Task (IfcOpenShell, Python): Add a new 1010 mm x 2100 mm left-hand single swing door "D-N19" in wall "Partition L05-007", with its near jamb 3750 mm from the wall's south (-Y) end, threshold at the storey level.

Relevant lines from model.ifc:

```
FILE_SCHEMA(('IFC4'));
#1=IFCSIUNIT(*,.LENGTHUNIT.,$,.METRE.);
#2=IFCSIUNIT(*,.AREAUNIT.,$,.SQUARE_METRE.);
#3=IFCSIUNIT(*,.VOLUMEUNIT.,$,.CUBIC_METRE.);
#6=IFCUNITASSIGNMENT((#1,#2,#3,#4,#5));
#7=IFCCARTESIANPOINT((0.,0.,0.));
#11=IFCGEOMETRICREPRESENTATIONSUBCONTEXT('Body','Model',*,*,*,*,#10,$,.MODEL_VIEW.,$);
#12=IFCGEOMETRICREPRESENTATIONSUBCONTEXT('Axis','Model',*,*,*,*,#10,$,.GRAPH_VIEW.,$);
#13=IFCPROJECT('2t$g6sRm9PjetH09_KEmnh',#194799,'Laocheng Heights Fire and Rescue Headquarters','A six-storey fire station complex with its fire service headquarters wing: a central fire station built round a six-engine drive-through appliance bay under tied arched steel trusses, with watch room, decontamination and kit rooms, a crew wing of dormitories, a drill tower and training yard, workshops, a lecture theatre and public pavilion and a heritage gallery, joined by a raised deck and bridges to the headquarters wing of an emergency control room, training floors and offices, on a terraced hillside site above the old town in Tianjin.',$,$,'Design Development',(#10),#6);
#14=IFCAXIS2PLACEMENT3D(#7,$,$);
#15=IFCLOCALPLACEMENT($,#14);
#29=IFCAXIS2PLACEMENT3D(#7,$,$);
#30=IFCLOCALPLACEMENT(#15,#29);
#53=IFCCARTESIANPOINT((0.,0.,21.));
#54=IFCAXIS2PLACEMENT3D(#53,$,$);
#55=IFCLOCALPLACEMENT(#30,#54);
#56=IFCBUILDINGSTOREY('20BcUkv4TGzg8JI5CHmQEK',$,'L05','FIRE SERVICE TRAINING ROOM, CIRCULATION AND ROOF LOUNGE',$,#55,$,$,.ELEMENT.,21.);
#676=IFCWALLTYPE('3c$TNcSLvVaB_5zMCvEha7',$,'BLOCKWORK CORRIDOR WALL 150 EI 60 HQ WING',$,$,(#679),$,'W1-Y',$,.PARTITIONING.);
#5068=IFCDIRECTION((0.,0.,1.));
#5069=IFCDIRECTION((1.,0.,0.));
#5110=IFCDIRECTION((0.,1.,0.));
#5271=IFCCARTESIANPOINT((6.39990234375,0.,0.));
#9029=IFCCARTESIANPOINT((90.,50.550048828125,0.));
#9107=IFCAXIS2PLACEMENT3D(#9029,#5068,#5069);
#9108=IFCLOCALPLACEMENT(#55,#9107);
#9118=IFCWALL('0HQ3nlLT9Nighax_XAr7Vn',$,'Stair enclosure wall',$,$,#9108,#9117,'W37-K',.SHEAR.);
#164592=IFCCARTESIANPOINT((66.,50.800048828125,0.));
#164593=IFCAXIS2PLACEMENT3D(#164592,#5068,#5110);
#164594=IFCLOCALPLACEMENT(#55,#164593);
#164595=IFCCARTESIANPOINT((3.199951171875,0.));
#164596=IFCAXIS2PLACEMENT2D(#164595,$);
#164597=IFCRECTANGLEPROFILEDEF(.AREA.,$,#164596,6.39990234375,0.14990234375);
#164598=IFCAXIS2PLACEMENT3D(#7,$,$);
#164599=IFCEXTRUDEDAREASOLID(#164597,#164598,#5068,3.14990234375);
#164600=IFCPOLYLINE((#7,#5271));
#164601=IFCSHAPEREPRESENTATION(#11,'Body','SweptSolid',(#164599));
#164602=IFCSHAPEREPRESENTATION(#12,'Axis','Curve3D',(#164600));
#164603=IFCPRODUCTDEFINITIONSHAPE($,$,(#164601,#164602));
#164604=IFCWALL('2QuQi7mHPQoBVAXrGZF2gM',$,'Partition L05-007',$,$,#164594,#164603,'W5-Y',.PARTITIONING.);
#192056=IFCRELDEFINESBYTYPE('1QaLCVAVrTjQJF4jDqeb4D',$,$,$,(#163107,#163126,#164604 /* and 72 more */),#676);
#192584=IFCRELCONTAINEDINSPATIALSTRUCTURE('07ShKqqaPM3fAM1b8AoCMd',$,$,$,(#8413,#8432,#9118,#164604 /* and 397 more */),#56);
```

```python
import numpy as np
import ifcopenshell
import ifcopenshell.api.feature
import ifcopenshell.api.geometry
import ifcopenshell.api.root
import ifcopenshell.api.spatial
import ifcopenshell.geom
import ifcopenshell.util.element
import ifcopenshell.util.placement
import ifcopenshell.util.representation
import ifcopenshell.util.shape
import ifcopenshell.util.unit

model = ifcopenshell.open("model.ifc")
unit_scale = ifcopenshell.util.unit.calculate_unit_scale(model)
settings = ifcopenshell.geom.settings()


def volume(element):
    """Net volume in cubic metres, openings subtracted."""
    shape = ifcopenshell.geom.create_shape(settings, element)
    return ifcopenshell.util.shape.get_volume(shape.geometry)


wall = model.by_guid("2QuQi7mHPQoBVAXrGZF2gM")
storey = ifcopenshell.util.element.get_container(wall, ifc_class="IfcBuildingStorey")
context = ifcopenshell.util.representation.get_context(model, "Model", "Body", "MODEL_VIEW")
before = volume(wall)

width, height, from_end, sill = 1.01, 2.1, 3.75, 0.0  # metres

# The wall runs along its own X axis, and the end named is its -X end.
wall_shape = ifcopenshell.geom.create_shape(settings, wall)
x, y, z = ifcopenshell.util.shape.get_vertices(wall_shape.geometry).T
start = x.min() + from_end
face, thickness = float(y.min()), float(y.max() - y.min())
wall_matrix = ifcopenshell.util.placement.get_local_placement(wall.ObjectPlacement)
level = ifcopenshell.util.placement.get_local_placement(storey.ObjectPlacement)[2, 3]


def in_wall(x, y):
    """Placement at x, y metres in the wall's axes, at sill height."""
    matrix = wall_matrix.copy()
    matrix[:, 3] = wall_matrix @ np.array([x / unit_scale, y / unit_scale, 0.0, 1.0])
    matrix[2, 3] = level + sill / unit_scale
    return matrix


# Opening: a box that overshoots both wall faces by 50 mm.
opening = ifcopenshell.api.root.create_entity(model, ifc_class="IfcOpeningElement", predefined_type="OPENING")
box = ifcopenshell.api.geometry.add_wall_representation(
    model, context=context, length=width, height=height, thickness=thickness + 0.1
)
ifcopenshell.api.geometry.assign_representation(model, product=opening, representation=box)
ifcopenshell.api.geometry.edit_object_placement(model, product=opening, matrix=in_wall(start, face - 0.05), is_si=False)
ifcopenshell.api.feature.add_feature(model, feature=opening, element=wall)

door = ifcopenshell.api.root.create_entity(model, ifc_class="IfcDoor", name="D-N19", predefined_type="DOOR")
door.OverallWidth, door.OverallHeight = width / unit_scale, height / unit_scale
door.OperationType = "SINGLE_SWING_LEFT"
body = ifcopenshell.api.geometry.add_door_representation(
    model,
    context=context,
    overall_width=door.OverallWidth,
    overall_height=door.OverallHeight,
    operation_type="SINGLE_SWING_LEFT",
    lining_properties={"LiningDepth": thickness / unit_scale, "ThresholdDepth": thickness / unit_scale},
)
ifcopenshell.api.geometry.assign_representation(model, product=door, representation=body)
ifcopenshell.api.spatial.assign_container(model, products=[door], relating_structure=storey)
ifcopenshell.api.feature.add_filling(model, opening=opening, element=door)

# The lining spans the wall, so the door starts at the wall face.
ifcopenshell.api.geometry.edit_object_placement(model, product=door, matrix=in_wall(start, face), is_si=False)

after = volume(wall)

print(f"wall volume {before:.3f} -> {after:.3f} m3")

model.write("model_rev.ifc")
```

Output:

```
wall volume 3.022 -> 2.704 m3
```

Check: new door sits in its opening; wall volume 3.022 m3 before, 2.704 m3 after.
